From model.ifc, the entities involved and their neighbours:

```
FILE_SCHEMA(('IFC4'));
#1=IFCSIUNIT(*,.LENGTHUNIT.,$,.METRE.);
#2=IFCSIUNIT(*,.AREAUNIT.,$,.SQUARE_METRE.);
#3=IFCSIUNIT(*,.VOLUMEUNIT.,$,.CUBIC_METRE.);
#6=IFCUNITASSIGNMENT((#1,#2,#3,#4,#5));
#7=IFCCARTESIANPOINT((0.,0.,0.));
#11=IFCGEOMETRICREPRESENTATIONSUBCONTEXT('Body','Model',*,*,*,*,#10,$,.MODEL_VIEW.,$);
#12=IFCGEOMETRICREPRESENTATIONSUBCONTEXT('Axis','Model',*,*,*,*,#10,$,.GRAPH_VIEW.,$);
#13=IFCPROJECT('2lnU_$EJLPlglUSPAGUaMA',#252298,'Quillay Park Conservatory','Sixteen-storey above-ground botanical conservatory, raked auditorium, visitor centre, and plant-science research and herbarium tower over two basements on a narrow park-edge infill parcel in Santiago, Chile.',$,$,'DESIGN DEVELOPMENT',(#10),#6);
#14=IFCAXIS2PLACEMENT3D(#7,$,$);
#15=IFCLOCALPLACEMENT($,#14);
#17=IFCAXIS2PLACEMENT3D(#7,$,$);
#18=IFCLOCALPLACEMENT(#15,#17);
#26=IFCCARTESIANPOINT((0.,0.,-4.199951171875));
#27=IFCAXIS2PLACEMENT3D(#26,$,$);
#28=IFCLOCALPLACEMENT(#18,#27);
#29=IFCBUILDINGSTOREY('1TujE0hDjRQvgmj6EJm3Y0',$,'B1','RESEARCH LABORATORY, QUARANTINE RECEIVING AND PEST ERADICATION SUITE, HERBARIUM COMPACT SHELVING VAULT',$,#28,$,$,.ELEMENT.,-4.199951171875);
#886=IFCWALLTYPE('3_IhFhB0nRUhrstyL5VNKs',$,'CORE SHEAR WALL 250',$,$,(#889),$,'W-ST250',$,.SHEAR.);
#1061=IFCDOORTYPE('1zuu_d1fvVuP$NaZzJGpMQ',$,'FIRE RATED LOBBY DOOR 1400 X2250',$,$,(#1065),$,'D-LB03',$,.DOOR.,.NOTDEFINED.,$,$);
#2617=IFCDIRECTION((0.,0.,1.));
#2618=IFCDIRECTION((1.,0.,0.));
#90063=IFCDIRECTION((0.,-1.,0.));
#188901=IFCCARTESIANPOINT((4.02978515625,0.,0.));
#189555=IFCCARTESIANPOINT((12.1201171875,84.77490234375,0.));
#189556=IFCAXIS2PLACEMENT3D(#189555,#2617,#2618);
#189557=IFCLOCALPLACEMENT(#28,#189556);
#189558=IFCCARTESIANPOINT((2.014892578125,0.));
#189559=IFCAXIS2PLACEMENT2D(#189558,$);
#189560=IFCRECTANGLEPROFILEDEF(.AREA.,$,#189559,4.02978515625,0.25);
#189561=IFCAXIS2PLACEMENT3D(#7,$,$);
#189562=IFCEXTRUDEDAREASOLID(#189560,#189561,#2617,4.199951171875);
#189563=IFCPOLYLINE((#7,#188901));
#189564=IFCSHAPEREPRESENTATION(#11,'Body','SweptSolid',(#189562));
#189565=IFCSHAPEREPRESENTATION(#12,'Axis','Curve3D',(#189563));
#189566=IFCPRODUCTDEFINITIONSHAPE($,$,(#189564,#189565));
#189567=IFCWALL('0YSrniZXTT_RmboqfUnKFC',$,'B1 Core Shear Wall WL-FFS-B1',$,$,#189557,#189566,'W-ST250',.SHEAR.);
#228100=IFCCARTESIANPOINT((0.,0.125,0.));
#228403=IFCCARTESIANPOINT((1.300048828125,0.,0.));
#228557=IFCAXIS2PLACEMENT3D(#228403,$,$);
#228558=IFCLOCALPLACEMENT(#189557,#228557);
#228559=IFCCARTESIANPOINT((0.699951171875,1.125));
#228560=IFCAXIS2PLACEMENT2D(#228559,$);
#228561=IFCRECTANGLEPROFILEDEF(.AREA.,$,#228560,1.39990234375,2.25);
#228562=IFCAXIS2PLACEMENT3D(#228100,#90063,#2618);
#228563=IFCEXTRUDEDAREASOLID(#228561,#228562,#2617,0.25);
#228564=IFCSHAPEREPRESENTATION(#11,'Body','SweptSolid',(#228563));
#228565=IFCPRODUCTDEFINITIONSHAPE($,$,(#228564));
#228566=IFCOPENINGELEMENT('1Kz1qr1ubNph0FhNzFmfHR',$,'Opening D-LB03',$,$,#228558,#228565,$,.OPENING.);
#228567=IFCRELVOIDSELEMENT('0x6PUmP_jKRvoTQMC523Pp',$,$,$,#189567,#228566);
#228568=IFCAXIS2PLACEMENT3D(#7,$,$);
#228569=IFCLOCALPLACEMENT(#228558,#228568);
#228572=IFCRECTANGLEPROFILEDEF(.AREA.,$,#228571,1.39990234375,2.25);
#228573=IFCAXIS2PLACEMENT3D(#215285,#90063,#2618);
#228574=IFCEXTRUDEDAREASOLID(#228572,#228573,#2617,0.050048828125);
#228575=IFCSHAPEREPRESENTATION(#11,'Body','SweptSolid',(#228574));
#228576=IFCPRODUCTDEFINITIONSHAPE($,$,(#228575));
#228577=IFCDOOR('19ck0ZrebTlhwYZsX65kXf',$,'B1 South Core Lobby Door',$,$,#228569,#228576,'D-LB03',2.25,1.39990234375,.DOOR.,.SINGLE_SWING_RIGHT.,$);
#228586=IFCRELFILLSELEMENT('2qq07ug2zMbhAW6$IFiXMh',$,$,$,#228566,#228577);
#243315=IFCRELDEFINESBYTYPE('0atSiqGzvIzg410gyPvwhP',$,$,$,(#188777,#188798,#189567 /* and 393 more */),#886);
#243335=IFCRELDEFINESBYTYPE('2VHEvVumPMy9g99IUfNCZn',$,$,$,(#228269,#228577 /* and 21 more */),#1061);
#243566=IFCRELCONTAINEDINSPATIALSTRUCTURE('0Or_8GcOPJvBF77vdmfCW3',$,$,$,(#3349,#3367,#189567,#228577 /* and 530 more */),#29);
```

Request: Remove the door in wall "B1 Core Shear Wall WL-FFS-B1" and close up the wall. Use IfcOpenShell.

```python
import ifcopenshell
import ifcopenshell.api.feature
import ifcopenshell.api.root
import ifcopenshell.geom
import ifcopenshell.util.shape

model = ifcopenshell.open("model.ifc")
settings = ifcopenshell.geom.settings()


def volume(element):
    """Net volume in cubic metres, openings subtracted."""
    shape = ifcopenshell.geom.create_shape(settings, element)
    return ifcopenshell.util.shape.get_volume(shape.geometry)


door = model.by_id(228577)
opening = door.FillsVoids[0].RelatingOpeningElement
wall = opening.VoidsElements[0].RelatingBuildingElement
before = volume(wall)

ifcopenshell.api.root.remove_product(model, product=door)
ifcopenshell.api.feature.remove_feature(model, feature=opening)

after = volume(wall)

print(f"wall volume {before:.3f} -> {after:.3f} m3")

model.write("model_edited.ifc")
```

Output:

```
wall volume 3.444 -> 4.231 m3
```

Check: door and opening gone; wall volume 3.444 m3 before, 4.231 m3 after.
